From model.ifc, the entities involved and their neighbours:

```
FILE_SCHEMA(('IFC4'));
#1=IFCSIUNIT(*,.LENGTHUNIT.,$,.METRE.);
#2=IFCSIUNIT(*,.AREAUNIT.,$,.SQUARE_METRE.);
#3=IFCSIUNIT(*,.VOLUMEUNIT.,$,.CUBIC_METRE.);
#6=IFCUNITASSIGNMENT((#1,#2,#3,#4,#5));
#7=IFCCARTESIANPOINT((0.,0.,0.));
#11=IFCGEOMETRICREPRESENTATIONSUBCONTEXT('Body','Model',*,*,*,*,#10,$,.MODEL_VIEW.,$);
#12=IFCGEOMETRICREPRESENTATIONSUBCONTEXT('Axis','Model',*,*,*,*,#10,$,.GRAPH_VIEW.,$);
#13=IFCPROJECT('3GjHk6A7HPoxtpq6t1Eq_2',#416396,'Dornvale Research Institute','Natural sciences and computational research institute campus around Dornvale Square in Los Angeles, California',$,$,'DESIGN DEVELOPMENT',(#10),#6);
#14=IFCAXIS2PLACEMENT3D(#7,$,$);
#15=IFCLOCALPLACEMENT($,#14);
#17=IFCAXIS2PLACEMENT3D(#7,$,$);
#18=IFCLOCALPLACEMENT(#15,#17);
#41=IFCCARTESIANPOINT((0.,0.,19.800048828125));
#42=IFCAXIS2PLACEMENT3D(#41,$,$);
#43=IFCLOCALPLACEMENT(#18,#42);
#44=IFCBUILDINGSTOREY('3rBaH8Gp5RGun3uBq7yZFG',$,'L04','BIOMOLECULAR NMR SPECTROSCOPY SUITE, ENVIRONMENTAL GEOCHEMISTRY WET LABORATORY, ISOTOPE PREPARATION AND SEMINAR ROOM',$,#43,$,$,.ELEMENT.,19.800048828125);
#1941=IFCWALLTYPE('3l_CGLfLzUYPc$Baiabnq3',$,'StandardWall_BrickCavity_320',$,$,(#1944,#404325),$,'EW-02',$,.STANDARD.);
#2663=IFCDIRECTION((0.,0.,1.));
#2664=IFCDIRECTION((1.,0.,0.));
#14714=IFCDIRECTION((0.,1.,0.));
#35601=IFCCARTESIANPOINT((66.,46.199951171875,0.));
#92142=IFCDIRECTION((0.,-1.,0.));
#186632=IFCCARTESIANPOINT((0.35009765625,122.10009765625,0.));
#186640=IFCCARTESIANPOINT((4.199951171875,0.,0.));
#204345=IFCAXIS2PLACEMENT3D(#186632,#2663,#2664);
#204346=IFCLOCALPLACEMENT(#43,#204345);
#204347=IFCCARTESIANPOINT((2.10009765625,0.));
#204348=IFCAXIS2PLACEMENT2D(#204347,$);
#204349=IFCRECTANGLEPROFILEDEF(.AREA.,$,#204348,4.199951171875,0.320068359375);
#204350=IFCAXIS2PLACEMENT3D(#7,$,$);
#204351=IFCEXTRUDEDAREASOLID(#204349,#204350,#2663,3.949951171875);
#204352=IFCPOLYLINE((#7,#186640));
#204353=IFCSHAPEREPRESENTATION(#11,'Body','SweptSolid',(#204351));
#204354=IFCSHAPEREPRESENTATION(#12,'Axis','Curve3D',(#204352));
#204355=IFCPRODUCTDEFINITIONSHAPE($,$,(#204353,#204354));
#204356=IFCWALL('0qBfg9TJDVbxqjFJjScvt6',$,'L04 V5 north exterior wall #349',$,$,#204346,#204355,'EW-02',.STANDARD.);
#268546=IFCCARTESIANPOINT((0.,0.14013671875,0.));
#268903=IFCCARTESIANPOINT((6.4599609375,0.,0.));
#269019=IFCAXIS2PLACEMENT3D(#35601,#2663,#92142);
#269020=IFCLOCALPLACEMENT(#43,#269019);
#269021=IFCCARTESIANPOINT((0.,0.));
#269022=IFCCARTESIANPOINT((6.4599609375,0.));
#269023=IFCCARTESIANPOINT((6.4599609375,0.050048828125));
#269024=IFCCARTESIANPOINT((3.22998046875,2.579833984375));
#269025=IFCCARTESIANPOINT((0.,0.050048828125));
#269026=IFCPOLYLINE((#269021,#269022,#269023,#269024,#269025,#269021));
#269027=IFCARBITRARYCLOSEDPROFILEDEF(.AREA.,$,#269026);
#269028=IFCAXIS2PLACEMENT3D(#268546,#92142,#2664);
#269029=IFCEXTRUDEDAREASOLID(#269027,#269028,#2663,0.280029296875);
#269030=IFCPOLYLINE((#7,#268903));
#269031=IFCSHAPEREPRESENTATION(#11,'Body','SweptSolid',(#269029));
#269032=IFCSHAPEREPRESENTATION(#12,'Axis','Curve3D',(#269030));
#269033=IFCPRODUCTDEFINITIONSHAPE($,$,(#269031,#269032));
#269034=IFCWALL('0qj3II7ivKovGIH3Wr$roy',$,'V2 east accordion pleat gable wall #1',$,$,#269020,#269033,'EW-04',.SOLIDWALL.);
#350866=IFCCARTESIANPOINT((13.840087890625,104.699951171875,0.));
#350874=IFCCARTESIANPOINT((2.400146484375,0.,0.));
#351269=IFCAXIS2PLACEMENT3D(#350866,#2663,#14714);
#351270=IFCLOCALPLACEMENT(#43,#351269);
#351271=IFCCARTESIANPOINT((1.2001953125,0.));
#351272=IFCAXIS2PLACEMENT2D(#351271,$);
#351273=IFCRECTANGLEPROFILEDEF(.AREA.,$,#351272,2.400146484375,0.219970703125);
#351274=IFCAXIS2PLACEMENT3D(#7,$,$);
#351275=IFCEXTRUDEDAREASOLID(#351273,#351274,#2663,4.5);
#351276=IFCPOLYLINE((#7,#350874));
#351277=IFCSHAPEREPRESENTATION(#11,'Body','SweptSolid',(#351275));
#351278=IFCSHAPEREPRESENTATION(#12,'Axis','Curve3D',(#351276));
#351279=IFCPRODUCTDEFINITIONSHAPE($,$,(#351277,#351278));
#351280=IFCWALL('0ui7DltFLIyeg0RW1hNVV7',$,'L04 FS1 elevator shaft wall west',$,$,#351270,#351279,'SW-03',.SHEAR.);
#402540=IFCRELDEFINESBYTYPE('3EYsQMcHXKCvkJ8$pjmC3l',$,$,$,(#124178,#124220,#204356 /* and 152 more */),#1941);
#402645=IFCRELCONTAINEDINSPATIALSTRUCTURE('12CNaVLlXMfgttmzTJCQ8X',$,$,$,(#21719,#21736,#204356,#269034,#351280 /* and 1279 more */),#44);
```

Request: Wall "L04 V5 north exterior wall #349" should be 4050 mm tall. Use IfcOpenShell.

```python
import ifcopenshell
import ifcopenshell.geom
import ifcopenshell.util.representation
import ifcopenshell.util.shape
import ifcopenshell.util.unit

model = ifcopenshell.open("model.ifc")
unit_scale = ifcopenshell.util.unit.calculate_unit_scale(model)
settings = ifcopenshell.geom.settings()


def volume(element):
    """Net volume in cubic metres, openings subtracted."""
    shape = ifcopenshell.geom.create_shape(settings, element)
    return ifcopenshell.util.shape.get_volume(shape.geometry)


wall = model.by_guid("0qBfg9TJDVbxqjFJjScvt6")
before = volume(wall)

body = ifcopenshell.util.representation.get_representation(wall, "Model", "Body")
solid = body.Items[0]
old_height = solid.Depth
solid.Depth = 4.05 / unit_scale
after = volume(wall)

print(f"height {old_height:g} -> {solid.Depth:g}, volume {before:.3f} -> {after:.3f} m3")

model.write("model_edited.ifc")
```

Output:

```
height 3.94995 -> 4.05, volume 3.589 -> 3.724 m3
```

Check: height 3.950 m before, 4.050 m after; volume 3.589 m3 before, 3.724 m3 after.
